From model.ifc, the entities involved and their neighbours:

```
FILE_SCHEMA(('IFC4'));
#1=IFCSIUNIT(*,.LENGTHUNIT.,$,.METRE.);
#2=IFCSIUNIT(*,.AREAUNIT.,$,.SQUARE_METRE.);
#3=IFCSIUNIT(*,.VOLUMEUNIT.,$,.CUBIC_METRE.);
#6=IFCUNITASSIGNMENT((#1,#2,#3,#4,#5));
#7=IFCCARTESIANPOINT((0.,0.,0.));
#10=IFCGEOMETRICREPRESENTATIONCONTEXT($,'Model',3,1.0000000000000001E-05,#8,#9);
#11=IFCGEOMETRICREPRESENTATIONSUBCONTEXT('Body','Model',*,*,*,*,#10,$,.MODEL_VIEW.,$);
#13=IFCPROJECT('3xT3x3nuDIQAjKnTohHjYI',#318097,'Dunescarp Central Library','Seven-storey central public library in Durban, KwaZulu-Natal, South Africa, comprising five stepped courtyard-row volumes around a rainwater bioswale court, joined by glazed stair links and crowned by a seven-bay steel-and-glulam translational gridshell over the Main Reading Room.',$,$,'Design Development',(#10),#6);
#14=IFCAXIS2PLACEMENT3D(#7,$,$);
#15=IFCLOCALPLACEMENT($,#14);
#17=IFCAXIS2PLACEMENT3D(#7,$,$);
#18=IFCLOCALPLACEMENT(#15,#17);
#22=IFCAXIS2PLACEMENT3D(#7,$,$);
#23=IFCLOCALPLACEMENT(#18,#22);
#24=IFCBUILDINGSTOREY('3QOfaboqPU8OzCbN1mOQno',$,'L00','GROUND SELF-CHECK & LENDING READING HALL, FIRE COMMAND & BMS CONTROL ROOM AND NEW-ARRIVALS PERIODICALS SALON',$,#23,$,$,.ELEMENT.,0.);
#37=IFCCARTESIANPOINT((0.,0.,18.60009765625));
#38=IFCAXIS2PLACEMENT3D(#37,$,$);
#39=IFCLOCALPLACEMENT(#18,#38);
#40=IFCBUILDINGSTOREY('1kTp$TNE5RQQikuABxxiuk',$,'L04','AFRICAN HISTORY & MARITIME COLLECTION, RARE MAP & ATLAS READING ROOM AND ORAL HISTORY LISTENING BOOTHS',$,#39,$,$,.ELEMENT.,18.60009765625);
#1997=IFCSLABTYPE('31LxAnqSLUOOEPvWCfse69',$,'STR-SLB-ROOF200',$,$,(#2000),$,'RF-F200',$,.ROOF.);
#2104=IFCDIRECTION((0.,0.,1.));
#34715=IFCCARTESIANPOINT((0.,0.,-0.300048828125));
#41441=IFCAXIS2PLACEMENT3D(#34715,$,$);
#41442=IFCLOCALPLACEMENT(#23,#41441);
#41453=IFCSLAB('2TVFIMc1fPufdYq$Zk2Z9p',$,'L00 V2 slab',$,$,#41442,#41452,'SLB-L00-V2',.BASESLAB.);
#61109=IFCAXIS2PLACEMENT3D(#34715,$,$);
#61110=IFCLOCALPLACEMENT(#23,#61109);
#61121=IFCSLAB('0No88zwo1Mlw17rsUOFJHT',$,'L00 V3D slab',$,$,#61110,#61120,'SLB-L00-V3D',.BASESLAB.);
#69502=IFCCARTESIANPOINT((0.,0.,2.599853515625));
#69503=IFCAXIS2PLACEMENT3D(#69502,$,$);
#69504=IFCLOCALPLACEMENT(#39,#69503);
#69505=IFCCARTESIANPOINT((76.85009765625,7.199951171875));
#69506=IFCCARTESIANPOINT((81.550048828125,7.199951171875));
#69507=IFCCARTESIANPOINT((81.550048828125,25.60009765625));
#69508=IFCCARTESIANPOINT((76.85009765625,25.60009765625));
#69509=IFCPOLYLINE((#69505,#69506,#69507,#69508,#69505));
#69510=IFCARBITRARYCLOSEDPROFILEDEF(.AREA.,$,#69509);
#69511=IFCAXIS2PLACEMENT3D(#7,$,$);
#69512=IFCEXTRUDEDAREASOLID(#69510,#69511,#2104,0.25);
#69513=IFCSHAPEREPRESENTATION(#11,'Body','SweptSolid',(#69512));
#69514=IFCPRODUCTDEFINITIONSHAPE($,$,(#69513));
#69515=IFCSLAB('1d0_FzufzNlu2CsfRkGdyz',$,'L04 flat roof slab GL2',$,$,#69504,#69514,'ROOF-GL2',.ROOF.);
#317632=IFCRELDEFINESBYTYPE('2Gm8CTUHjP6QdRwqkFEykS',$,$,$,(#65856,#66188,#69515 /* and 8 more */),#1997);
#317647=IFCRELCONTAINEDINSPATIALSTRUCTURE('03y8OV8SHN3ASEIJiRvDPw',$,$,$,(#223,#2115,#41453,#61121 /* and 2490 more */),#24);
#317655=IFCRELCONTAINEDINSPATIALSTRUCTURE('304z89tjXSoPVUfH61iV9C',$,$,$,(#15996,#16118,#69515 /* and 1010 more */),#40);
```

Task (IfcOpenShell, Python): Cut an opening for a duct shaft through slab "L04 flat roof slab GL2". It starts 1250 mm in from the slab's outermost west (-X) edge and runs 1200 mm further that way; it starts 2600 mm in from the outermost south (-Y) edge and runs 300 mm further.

```python
import numpy as np
import ifcopenshell
import ifcopenshell.api.feature
import ifcopenshell.api.geometry
import ifcopenshell.api.root
import ifcopenshell.geom
import ifcopenshell.util.placement
import ifcopenshell.util.representation
import ifcopenshell.util.shape
import ifcopenshell.util.unit

model = ifcopenshell.open("model.ifc")
unit_scale = ifcopenshell.util.unit.calculate_unit_scale(model)
settings = ifcopenshell.geom.settings()


def volume(element):
    """Net volume in cubic metres, openings subtracted."""
    shape = ifcopenshell.geom.create_shape(settings, element)
    return ifcopenshell.util.shape.get_volume(shape.geometry)


slab = model.by_guid("1d0_FzufzNlu2CsfRkGdyz")
before = volume(slab)

# Extent in the slab's own axes, in metres. The edges named are its -X and -Y sides.
slab_shape = ifcopenshell.geom.create_shape(settings, slab)
vertices = ifcopenshell.util.shape.get_vertices(slab_shape.geometry)
x_min, y_min, bottom = vertices.min(axis=0)
top = vertices[:, 2].max()

opening = ifcopenshell.api.root.create_entity(model, ifc_class="IfcOpeningElement", name="Duct shaft opening", predefined_type="OPENING")
context = ifcopenshell.util.representation.get_context(model, "Model", "Body", "MODEL_VIEW")
width, depth = 1.2, 0.3
outline = [(0.0, 0.0), (width, 0.0), (width, depth), (0.0, depth), (0.0, 0.0)]
# Overshoot both faces by 50 mm so the cut is clean.
shape = ifcopenshell.api.geometry.add_slab_representation(
    model, context=context, depth=top - bottom + 0.1, polyline=outline
)
ifcopenshell.api.geometry.assign_representation(model, product=opening, representation=shape)

matrix = ifcopenshell.util.placement.get_local_placement(slab.ObjectPlacement)
matrix[:, 3] = matrix @ np.append(np.array([x_min + 1.25, y_min + 2.6, bottom - 0.05]) / unit_scale, 1.0)
ifcopenshell.api.geometry.edit_object_placement(model, product=opening, matrix=matrix, is_si=False)
ifcopenshell.api.feature.add_feature(model, feature=opening, element=slab)

after = volume(slab)

print(f"slab volume {before:.3f} -> {after:.3f} m3")

model.write("model_rev.ifc")
```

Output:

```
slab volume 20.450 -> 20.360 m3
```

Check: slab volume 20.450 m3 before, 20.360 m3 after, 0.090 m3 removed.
